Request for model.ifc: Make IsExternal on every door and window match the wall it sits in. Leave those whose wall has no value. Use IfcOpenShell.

First a look at what the model holds.

```python
import ifcopenshell
import ifcopenshell.util.element

model = ifcopenshell.open("model.ifc")
print(model.schema)
seen = {}
for e in model.by_type("IfcDoor") + model.by_type("IfcWindow"):
    if not e.FillsVoids:
        continue
    host = e.FillsVoids[0].RelatingOpeningElement.VoidsElements[0].RelatingBuildingElement
    own = ifcopenshell.util.element.get_pset(e, f"Pset_{e.is_a()[3:].removesuffix('StandardCase')}Common", "IsExternal")
    wall = ifcopenshell.util.element.get_pset(host, "Pset_WallCommon", "IsExternal")
    seen[e.is_a(), own, wall] = seen.get((e.is_a(), own, wall), 0) + 1
for (cls, own, wall), count in sorted(seen.items(), key=str):
    print(count, cls, "IsExternal:", own, "| host wall:", wall)
```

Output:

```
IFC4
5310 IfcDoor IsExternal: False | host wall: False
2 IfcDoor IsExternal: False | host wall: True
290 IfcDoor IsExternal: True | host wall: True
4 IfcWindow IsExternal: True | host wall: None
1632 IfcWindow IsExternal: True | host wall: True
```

```python
import ifcopenshell
import ifcopenshell.api.pset
import ifcopenshell.util.element

model = ifcopenshell.open("model.ifc")

count = 0
for ifc_class, pset_name in (("IfcDoor", "Pset_DoorCommon"), ("IfcWindow", "Pset_WindowCommon")):
    for e in model.by_type(ifc_class):
        if not e.FillsVoids:
            continue
        host = e.FillsVoids[0].RelatingOpeningElement.VoidsElements[0].RelatingBuildingElement
        external = ifcopenshell.util.element.get_pset(host, "Pset_WallCommon", "IsExternal")
        if external is None or ifcopenshell.util.element.get_pset(e, pset_name, "IsExternal") == external:
            continue
        found = ifcopenshell.util.element.get_pset(e, pset_name, should_inherit=False)
        if found:
            pset = model.by_id(found["id"])
            if len(ifcopenshell.util.element.get_elements_by_pset(pset)) > 1:
                pset = ifcopenshell.api.pset.unshare_pset(model, products=[e], pset=pset)[0]
        else:
            pset = ifcopenshell.api.pset.add_pset(model, product=e, name=pset_name)
        ifcopenshell.api.pset.edit_pset(model, pset=pset, properties={"IsExternal": external})
        count += 1

print(count, "updated")

model.write("model_rev.ifc")
```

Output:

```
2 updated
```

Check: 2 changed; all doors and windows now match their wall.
